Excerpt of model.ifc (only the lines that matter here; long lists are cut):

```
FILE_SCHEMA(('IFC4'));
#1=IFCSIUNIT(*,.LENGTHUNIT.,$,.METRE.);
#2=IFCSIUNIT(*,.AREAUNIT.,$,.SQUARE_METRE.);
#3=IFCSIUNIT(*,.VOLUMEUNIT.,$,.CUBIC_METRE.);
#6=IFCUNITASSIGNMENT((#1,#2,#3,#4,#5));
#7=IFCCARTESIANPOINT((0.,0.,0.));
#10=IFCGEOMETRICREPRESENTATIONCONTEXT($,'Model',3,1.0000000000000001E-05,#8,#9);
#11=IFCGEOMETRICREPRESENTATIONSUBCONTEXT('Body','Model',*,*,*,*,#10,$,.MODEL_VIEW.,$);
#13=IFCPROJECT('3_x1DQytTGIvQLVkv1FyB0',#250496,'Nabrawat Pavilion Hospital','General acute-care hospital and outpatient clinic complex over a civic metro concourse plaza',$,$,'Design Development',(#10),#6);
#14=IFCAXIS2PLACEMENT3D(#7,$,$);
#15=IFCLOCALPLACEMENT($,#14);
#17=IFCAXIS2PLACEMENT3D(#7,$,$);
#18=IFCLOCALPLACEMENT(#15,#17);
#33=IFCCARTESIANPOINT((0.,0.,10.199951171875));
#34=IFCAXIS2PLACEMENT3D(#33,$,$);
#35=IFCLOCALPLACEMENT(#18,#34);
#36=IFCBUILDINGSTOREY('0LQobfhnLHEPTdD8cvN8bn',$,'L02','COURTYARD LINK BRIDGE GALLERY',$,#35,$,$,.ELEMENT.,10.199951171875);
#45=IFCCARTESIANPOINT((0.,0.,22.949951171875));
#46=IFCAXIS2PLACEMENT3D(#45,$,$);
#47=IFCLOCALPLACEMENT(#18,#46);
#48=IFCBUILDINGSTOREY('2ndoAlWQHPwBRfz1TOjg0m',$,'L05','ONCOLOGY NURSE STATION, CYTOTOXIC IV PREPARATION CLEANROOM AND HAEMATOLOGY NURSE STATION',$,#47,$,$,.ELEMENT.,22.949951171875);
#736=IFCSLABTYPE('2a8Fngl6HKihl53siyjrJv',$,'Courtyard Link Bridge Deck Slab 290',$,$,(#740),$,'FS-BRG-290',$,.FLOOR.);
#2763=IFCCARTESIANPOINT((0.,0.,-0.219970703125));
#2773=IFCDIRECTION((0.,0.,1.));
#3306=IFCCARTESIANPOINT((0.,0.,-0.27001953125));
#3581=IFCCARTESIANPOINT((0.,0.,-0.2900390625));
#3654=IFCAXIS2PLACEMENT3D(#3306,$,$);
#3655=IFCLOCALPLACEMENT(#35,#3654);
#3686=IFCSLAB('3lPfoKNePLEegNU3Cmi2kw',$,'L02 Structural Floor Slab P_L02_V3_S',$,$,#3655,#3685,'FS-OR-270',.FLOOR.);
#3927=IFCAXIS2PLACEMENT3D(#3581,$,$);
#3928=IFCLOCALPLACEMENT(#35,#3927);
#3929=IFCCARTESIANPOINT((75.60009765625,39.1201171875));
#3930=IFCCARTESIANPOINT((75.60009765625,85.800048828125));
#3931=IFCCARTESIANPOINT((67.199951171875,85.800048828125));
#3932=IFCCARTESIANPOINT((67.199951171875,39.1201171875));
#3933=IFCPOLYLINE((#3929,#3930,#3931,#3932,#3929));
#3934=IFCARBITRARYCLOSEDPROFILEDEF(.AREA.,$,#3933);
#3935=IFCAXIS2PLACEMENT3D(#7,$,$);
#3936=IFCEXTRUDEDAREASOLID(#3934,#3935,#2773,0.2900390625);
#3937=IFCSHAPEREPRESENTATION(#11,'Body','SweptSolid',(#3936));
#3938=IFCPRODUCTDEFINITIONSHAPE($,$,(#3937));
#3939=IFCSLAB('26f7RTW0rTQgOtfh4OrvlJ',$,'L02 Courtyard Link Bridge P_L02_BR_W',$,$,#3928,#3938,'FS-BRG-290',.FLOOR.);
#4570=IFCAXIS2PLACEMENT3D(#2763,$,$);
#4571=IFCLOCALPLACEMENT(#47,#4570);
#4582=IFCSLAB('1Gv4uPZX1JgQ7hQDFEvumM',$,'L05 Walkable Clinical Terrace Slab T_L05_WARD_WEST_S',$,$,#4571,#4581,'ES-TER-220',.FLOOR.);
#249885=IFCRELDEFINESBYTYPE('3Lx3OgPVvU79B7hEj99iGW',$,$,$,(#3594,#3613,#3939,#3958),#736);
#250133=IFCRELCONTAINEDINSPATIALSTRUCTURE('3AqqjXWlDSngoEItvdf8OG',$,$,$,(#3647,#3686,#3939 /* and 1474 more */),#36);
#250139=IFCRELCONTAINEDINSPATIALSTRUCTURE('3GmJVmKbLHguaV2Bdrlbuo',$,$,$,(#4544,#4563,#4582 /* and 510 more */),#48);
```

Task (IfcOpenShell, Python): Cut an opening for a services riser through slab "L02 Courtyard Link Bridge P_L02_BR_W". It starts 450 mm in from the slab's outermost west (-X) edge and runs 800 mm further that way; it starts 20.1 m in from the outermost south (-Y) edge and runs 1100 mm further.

```python
import numpy as np
import ifcopenshell
import ifcopenshell.api.feature
import ifcopenshell.api.geometry
import ifcopenshell.api.root
import ifcopenshell.geom
import ifcopenshell.util.placement
import ifcopenshell.util.representation
import ifcopenshell.util.shape
import ifcopenshell.util.unit

model = ifcopenshell.open("model.ifc")
unit_scale = ifcopenshell.util.unit.calculate_unit_scale(model)
settings = ifcopenshell.geom.settings()


def volume(element):
    """Net volume in cubic metres, openings subtracted."""
    shape = ifcopenshell.geom.create_shape(settings, element)
    return ifcopenshell.util.shape.get_volume(shape.geometry)


slab = model.by_guid("26f7RTW0rTQgOtfh4OrvlJ")
before = volume(slab)

# Extent in the slab's own axes, in metres. The edges named are its -X and -Y sides.
slab_shape = ifcopenshell.geom.create_shape(settings, slab)
vertices = ifcopenshell.util.shape.get_vertices(slab_shape.geometry)
x_min, y_min, bottom = vertices.min(axis=0)
top = vertices[:, 2].max()

opening = ifcopenshell.api.root.create_entity(model, ifc_class="IfcOpeningElement", name="Services riser opening", predefined_type="OPENING")
context = ifcopenshell.util.representation.get_context(model, "Model", "Body", "MODEL_VIEW")
width, depth = 0.8, 1.1
outline = [(0.0, 0.0), (width, 0.0), (width, depth), (0.0, depth), (0.0, 0.0)]
# Overshoot both faces by 50 mm so the cut is clean.
shape = ifcopenshell.api.geometry.add_slab_representation(
    model, context=context, depth=top - bottom + 0.1, polyline=outline
)
ifcopenshell.api.geometry.assign_representation(model, product=opening, representation=shape)

matrix = ifcopenshell.util.placement.get_local_placement(slab.ObjectPlacement)
matrix[:, 3] = matrix @ np.append(np.array([x_min + 0.45, y_min + 20.1, bottom - 0.05]) / unit_scale, 1.0)
ifcopenshell.api.geometry.edit_object_placement(model, product=opening, matrix=matrix, is_si=False)
ifcopenshell.api.feature.add_feature(model, feature=opening, element=slab)

after = volume(slab)

print(f"slab volume {before:.3f} -> {after:.3f} m3")

model.write("model_edited.ifc")
```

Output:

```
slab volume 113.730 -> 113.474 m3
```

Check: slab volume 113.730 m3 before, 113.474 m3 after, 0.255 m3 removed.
